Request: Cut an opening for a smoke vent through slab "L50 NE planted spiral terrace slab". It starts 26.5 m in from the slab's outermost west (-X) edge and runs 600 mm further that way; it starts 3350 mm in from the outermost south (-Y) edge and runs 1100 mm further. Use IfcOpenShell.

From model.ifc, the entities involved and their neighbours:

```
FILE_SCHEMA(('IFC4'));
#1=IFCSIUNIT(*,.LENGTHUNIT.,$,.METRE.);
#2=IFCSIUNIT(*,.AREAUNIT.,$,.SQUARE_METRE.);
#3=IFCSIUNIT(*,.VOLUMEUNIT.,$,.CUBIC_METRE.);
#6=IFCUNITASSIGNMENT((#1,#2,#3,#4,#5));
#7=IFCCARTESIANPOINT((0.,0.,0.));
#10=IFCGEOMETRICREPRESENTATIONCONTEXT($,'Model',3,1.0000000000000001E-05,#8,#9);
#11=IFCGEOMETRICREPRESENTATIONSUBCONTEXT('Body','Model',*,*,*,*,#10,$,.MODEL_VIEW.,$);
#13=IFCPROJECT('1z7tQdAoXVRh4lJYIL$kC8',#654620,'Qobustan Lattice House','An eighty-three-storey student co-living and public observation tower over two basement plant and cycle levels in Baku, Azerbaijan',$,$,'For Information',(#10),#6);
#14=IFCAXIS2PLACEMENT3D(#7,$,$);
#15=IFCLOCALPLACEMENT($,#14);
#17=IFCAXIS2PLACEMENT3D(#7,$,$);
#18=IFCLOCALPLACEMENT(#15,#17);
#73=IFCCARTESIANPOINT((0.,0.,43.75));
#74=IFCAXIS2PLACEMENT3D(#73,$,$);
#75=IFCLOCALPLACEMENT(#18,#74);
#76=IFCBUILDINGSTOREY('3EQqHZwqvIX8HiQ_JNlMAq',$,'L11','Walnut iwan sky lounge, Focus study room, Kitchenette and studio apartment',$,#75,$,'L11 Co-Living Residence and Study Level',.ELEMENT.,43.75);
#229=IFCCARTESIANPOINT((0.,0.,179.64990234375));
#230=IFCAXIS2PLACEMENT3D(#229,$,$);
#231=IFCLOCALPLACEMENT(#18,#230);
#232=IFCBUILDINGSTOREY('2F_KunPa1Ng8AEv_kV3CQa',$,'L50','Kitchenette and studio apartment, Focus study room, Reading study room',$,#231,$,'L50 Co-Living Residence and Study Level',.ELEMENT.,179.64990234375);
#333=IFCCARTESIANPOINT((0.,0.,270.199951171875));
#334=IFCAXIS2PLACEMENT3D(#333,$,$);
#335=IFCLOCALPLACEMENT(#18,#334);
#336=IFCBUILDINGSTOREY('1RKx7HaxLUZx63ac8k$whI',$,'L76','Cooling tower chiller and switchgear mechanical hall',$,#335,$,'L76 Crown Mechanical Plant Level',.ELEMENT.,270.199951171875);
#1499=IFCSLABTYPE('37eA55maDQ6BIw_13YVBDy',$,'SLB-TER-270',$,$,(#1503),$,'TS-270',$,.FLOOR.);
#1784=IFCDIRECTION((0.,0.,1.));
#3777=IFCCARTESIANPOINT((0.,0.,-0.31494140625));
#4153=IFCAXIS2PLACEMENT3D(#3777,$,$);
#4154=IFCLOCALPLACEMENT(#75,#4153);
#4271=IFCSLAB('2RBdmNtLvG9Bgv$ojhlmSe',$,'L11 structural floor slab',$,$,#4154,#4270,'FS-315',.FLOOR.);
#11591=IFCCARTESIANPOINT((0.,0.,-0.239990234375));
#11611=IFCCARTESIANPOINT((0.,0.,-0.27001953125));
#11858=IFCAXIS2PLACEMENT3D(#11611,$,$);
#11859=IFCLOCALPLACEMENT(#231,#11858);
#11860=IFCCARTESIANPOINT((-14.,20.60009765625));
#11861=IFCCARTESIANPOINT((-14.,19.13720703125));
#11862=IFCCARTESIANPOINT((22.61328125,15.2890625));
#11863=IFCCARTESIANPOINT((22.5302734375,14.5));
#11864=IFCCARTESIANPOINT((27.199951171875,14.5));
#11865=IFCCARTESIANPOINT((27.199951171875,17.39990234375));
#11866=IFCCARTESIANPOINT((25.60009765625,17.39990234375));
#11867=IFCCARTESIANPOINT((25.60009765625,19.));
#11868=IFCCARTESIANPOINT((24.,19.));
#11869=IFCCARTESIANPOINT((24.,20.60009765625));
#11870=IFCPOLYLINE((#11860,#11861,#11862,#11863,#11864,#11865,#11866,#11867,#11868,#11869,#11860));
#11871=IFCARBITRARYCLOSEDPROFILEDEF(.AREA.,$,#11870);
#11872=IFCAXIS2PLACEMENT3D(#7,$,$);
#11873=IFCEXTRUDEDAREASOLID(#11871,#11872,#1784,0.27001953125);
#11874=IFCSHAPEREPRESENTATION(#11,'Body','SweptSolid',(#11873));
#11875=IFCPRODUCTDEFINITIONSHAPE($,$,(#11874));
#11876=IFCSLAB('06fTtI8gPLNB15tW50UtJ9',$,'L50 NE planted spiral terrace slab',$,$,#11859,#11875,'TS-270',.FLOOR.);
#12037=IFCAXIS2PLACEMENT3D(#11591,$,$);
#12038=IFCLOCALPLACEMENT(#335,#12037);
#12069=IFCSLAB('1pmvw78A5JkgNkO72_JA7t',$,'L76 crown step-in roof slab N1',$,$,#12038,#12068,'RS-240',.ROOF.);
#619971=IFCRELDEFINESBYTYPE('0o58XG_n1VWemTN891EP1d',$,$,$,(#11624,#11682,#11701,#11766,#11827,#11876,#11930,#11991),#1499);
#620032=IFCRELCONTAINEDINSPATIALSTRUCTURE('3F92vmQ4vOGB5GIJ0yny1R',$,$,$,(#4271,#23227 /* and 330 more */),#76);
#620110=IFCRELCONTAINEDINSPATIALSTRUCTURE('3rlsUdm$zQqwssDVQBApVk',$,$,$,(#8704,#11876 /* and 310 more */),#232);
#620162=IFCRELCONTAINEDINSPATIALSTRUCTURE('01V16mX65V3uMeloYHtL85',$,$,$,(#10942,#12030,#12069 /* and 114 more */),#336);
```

```python
import numpy as np
import ifcopenshell
import ifcopenshell.api.feature
import ifcopenshell.api.geometry
import ifcopenshell.api.root
import ifcopenshell.geom
import ifcopenshell.util.placement
import ifcopenshell.util.representation
import ifcopenshell.util.shape
import ifcopenshell.util.unit

model = ifcopenshell.open("model.ifc")
unit_scale = ifcopenshell.util.unit.calculate_unit_scale(model)
settings = ifcopenshell.geom.settings()


def volume(element):
    """Net volume in cubic metres, openings subtracted."""
    shape = ifcopenshell.geom.create_shape(settings, element)
    return ifcopenshell.util.shape.get_volume(shape.geometry)


slab = model.by_guid("06fTtI8gPLNB15tW50UtJ9")
before = volume(slab)

# Extent in the slab's own axes, in metres. The edges named are its -X and -Y sides.
slab_shape = ifcopenshell.geom.create_shape(settings, slab)
vertices = ifcopenshell.util.shape.get_vertices(slab_shape.geometry)
x_min, y_min, bottom = vertices.min(axis=0)
top = vertices[:, 2].max()

opening = ifcopenshell.api.root.create_entity(model, ifc_class="IfcOpeningElement", name="Smoke vent opening", predefined_type="OPENING")
context = ifcopenshell.util.representation.get_context(model, "Model", "Body", "MODEL_VIEW")
width, depth = 0.6, 1.1
outline = [(0.0, 0.0), (width, 0.0), (width, depth), (0.0, depth), (0.0, 0.0)]
# Overshoot both faces by 50 mm so the cut is clean.
shape = ifcopenshell.api.geometry.add_slab_representation(
    model, context=context, depth=top - bottom + 0.1, polyline=outline
)
ifcopenshell.api.geometry.assign_representation(model, product=opening, representation=shape)

matrix = ifcopenshell.util.placement.get_local_placement(slab.ObjectPlacement)
matrix[:, 3] = matrix @ np.append(np.array([x_min + 26.5, y_min + 3.35, bottom - 0.05]) / unit_scale, 1.0)
ifcopenshell.api.geometry.edit_object_placement(model, product=opening, matrix=matrix, is_si=False)
ifcopenshell.api.feature.add_feature(model, feature=opening, element=slab)

after = volume(slab)

print(f"slab volume {before:.3f} -> {after:.3f} m3")

model.write("model_v2.ifc")
```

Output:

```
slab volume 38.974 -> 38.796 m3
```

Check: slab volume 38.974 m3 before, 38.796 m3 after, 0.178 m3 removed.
